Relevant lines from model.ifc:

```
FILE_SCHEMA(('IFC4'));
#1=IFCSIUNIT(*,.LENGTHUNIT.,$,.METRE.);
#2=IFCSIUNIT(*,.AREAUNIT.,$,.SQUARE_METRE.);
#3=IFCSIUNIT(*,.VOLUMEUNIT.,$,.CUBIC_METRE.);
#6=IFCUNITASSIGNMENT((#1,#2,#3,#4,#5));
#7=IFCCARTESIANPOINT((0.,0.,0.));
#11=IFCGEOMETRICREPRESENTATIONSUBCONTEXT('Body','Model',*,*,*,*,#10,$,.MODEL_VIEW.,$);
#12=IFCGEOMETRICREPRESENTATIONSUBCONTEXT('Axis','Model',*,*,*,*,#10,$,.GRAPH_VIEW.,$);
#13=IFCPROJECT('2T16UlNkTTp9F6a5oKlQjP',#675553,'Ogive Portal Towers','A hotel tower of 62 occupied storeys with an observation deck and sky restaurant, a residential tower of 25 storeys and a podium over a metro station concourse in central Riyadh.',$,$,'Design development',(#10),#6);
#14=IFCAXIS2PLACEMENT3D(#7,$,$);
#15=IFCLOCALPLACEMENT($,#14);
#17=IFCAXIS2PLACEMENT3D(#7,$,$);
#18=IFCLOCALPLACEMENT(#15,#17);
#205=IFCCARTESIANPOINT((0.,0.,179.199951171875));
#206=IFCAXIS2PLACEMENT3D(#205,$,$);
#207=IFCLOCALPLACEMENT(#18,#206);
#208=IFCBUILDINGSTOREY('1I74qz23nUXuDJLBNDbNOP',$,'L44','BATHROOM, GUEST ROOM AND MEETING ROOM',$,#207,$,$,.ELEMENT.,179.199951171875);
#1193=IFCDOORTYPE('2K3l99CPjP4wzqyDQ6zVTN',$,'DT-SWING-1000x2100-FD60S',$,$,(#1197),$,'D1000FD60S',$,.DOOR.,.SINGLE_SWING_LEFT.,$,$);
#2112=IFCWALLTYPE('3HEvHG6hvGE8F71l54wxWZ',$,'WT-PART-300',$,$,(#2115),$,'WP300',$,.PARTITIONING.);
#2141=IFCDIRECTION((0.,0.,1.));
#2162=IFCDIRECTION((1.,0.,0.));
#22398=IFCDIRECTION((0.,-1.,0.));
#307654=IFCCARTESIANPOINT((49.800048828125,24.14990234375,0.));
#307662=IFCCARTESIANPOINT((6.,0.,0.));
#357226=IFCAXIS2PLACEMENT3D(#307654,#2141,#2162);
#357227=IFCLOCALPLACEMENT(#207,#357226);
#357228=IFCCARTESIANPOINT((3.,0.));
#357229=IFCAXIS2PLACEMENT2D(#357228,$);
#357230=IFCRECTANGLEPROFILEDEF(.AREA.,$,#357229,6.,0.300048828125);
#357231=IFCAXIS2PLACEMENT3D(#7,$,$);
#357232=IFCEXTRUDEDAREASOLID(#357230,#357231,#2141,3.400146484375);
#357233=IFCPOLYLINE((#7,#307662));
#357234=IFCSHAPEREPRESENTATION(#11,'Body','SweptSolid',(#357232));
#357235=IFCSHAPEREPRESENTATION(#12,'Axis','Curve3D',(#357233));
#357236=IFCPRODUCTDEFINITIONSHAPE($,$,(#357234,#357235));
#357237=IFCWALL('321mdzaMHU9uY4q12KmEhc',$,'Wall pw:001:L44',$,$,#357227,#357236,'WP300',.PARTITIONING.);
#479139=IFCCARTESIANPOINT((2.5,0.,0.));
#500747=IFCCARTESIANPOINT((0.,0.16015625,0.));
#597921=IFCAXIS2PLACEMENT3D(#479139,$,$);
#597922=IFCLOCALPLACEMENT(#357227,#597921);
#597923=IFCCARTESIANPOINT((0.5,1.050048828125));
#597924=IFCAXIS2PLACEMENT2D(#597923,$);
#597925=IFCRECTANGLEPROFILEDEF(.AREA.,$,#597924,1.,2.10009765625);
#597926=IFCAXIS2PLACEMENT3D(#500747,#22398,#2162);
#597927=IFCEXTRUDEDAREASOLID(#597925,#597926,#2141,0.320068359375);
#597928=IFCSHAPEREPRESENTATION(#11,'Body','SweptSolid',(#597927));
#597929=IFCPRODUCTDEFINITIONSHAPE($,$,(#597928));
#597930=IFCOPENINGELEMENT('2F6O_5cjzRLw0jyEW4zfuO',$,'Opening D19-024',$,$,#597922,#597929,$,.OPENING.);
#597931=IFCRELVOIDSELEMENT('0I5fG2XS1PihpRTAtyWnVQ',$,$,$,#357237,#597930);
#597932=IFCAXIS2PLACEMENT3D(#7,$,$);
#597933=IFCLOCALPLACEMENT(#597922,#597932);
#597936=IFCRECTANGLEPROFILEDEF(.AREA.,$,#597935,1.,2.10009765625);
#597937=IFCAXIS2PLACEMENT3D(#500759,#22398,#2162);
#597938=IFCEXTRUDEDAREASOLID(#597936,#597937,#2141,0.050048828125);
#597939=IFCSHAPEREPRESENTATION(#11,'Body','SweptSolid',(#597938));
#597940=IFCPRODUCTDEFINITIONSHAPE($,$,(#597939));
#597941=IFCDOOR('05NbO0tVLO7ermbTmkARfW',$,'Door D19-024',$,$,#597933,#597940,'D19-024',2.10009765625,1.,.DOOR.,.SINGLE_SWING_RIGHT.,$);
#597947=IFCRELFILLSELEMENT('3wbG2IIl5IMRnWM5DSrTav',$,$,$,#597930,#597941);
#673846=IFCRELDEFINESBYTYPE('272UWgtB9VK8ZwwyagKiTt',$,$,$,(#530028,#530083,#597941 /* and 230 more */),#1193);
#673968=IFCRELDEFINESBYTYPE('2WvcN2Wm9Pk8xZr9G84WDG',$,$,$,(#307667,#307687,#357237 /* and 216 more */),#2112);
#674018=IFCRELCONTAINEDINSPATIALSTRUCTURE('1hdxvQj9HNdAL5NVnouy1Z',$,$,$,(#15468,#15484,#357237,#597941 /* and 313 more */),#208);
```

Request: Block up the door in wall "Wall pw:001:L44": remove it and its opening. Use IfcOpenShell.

```python
import ifcopenshell
import ifcopenshell.api.feature
import ifcopenshell.api.root
import ifcopenshell.geom
import ifcopenshell.util.shape

model = ifcopenshell.open("model.ifc")
settings = ifcopenshell.geom.settings()


def volume(element):
    """Net volume in cubic metres, openings subtracted."""
    shape = ifcopenshell.geom.create_shape(settings, element)
    return ifcopenshell.util.shape.get_volume(shape.geometry)


door = model.by_guid("05NbO0tVLO7ermbTmkARfW")
opening = door.FillsVoids[0].RelatingOpeningElement
wall = opening.VoidsElements[0].RelatingBuildingElement
before = volume(wall)

ifcopenshell.api.root.remove_product(model, product=door)
ifcopenshell.api.feature.remove_feature(model, feature=opening)

after = volume(wall)

print(f"wall volume {before:.3f} -> {after:.3f} m3")

model.write("model_v2.ifc")
```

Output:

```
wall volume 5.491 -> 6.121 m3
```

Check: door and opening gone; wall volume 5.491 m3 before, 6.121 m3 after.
